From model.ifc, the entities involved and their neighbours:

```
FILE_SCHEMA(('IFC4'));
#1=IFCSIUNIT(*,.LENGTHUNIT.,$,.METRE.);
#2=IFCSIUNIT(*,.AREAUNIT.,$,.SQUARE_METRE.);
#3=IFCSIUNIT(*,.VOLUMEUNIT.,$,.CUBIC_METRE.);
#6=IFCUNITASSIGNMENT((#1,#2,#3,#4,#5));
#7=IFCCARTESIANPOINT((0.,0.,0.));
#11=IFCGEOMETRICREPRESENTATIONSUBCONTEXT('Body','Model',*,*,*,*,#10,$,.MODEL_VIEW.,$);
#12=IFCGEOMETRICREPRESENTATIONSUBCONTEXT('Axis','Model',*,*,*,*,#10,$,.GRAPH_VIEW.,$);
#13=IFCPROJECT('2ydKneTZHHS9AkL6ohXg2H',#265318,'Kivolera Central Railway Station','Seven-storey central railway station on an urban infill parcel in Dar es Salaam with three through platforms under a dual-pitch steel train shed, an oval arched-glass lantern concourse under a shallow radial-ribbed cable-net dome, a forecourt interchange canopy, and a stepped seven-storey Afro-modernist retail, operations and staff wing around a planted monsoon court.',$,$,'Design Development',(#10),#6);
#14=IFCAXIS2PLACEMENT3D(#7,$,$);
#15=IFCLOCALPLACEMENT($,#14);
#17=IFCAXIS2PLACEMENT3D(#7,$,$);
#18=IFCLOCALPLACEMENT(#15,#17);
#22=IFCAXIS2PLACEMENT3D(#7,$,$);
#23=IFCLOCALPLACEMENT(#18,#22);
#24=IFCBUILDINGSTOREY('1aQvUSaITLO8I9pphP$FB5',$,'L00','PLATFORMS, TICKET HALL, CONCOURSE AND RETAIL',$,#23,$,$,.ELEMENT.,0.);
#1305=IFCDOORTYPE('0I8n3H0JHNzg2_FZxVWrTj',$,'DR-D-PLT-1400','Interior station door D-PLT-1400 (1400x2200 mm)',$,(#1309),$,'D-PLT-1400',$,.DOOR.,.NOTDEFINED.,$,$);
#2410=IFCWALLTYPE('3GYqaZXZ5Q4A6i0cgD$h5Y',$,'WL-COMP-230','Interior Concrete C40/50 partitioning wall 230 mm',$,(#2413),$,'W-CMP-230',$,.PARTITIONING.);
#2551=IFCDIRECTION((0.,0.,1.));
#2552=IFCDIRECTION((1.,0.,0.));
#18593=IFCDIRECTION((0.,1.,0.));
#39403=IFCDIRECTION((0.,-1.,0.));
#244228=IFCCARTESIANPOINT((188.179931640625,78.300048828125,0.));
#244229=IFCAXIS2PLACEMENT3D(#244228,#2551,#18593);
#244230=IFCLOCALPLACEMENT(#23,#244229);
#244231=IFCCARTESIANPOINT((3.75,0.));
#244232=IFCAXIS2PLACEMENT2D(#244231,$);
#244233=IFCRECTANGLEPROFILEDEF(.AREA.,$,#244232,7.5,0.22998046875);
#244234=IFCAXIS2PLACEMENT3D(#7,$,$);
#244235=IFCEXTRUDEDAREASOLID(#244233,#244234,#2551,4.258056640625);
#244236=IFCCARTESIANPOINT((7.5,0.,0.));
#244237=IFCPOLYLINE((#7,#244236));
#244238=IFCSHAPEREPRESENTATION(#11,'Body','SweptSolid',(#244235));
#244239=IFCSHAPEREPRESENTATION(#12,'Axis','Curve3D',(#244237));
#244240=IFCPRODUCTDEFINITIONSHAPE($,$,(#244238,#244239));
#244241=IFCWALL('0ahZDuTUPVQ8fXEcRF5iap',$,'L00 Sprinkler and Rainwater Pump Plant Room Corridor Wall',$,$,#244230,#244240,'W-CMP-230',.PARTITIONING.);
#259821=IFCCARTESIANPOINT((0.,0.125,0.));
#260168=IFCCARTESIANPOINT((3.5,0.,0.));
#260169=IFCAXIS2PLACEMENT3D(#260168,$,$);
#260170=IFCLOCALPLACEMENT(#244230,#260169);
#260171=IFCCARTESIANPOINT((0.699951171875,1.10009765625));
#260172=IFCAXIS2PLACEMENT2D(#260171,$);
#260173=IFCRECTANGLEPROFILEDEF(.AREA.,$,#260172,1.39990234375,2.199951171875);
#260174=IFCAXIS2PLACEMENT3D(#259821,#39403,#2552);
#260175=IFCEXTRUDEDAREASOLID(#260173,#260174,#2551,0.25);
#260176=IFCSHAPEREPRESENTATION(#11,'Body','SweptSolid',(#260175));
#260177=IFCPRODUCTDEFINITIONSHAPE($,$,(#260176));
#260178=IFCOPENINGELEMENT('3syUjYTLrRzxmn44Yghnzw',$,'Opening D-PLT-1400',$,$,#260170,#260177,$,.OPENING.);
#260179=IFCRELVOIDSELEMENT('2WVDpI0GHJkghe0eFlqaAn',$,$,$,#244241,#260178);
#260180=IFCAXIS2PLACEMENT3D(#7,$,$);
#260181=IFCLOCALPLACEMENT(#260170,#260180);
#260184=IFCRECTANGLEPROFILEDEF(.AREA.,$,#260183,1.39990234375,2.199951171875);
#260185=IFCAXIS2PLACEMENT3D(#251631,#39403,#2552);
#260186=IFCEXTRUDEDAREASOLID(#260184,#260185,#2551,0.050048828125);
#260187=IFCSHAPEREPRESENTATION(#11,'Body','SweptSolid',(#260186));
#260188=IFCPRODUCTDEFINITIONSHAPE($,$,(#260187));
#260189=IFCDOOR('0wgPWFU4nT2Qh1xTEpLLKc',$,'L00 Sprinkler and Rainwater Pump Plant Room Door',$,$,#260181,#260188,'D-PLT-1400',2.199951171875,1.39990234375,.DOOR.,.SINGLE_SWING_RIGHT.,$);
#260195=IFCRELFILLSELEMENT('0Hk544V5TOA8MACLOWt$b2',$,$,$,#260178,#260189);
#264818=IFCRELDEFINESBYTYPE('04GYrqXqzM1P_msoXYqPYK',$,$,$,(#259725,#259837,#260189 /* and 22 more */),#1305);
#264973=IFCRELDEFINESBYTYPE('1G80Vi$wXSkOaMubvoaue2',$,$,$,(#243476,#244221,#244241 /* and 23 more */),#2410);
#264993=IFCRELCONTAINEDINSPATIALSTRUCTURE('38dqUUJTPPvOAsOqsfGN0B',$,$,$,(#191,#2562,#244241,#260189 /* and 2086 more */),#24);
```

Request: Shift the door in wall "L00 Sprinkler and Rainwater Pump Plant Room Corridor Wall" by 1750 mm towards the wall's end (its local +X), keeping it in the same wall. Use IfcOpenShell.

```python
import ifcopenshell
import ifcopenshell.api.geometry
import ifcopenshell.util.placement
import ifcopenshell.util.unit

model = ifcopenshell.open("model.ifc")
unit_scale = ifcopenshell.util.unit.calculate_unit_scale(model)

door = model.by_guid("0wgPWFU4nT2Qh1xTEpLLKc")
opening = door.FillsVoids[0].RelatingOpeningElement
wall = opening.VoidsElements[0].RelatingBuildingElement

wall_matrix = ifcopenshell.util.placement.get_local_placement(wall.ObjectPlacement)
shift = wall_matrix[:3, 0] * 1.75 / unit_scale
before = ifcopenshell.util.placement.get_local_placement(door.ObjectPlacement)[:3, 3].copy()

# The door is placed relative to its opening, so it follows when the opening moves.
matrix = ifcopenshell.util.placement.get_local_placement(opening.ObjectPlacement)
matrix[:3, 3] += shift
ifcopenshell.api.geometry.edit_object_placement(
    model, product=opening, matrix=matrix, is_si=False, should_transform_children=True
)

after = ifcopenshell.util.placement.get_local_placement(door.ObjectPlacement)[:3, 3]
print("door moved by", (after - before).round(3) + 0.0)

model.write("model-out.ifc")
```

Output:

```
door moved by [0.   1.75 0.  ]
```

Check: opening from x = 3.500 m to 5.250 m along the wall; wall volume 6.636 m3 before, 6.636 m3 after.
